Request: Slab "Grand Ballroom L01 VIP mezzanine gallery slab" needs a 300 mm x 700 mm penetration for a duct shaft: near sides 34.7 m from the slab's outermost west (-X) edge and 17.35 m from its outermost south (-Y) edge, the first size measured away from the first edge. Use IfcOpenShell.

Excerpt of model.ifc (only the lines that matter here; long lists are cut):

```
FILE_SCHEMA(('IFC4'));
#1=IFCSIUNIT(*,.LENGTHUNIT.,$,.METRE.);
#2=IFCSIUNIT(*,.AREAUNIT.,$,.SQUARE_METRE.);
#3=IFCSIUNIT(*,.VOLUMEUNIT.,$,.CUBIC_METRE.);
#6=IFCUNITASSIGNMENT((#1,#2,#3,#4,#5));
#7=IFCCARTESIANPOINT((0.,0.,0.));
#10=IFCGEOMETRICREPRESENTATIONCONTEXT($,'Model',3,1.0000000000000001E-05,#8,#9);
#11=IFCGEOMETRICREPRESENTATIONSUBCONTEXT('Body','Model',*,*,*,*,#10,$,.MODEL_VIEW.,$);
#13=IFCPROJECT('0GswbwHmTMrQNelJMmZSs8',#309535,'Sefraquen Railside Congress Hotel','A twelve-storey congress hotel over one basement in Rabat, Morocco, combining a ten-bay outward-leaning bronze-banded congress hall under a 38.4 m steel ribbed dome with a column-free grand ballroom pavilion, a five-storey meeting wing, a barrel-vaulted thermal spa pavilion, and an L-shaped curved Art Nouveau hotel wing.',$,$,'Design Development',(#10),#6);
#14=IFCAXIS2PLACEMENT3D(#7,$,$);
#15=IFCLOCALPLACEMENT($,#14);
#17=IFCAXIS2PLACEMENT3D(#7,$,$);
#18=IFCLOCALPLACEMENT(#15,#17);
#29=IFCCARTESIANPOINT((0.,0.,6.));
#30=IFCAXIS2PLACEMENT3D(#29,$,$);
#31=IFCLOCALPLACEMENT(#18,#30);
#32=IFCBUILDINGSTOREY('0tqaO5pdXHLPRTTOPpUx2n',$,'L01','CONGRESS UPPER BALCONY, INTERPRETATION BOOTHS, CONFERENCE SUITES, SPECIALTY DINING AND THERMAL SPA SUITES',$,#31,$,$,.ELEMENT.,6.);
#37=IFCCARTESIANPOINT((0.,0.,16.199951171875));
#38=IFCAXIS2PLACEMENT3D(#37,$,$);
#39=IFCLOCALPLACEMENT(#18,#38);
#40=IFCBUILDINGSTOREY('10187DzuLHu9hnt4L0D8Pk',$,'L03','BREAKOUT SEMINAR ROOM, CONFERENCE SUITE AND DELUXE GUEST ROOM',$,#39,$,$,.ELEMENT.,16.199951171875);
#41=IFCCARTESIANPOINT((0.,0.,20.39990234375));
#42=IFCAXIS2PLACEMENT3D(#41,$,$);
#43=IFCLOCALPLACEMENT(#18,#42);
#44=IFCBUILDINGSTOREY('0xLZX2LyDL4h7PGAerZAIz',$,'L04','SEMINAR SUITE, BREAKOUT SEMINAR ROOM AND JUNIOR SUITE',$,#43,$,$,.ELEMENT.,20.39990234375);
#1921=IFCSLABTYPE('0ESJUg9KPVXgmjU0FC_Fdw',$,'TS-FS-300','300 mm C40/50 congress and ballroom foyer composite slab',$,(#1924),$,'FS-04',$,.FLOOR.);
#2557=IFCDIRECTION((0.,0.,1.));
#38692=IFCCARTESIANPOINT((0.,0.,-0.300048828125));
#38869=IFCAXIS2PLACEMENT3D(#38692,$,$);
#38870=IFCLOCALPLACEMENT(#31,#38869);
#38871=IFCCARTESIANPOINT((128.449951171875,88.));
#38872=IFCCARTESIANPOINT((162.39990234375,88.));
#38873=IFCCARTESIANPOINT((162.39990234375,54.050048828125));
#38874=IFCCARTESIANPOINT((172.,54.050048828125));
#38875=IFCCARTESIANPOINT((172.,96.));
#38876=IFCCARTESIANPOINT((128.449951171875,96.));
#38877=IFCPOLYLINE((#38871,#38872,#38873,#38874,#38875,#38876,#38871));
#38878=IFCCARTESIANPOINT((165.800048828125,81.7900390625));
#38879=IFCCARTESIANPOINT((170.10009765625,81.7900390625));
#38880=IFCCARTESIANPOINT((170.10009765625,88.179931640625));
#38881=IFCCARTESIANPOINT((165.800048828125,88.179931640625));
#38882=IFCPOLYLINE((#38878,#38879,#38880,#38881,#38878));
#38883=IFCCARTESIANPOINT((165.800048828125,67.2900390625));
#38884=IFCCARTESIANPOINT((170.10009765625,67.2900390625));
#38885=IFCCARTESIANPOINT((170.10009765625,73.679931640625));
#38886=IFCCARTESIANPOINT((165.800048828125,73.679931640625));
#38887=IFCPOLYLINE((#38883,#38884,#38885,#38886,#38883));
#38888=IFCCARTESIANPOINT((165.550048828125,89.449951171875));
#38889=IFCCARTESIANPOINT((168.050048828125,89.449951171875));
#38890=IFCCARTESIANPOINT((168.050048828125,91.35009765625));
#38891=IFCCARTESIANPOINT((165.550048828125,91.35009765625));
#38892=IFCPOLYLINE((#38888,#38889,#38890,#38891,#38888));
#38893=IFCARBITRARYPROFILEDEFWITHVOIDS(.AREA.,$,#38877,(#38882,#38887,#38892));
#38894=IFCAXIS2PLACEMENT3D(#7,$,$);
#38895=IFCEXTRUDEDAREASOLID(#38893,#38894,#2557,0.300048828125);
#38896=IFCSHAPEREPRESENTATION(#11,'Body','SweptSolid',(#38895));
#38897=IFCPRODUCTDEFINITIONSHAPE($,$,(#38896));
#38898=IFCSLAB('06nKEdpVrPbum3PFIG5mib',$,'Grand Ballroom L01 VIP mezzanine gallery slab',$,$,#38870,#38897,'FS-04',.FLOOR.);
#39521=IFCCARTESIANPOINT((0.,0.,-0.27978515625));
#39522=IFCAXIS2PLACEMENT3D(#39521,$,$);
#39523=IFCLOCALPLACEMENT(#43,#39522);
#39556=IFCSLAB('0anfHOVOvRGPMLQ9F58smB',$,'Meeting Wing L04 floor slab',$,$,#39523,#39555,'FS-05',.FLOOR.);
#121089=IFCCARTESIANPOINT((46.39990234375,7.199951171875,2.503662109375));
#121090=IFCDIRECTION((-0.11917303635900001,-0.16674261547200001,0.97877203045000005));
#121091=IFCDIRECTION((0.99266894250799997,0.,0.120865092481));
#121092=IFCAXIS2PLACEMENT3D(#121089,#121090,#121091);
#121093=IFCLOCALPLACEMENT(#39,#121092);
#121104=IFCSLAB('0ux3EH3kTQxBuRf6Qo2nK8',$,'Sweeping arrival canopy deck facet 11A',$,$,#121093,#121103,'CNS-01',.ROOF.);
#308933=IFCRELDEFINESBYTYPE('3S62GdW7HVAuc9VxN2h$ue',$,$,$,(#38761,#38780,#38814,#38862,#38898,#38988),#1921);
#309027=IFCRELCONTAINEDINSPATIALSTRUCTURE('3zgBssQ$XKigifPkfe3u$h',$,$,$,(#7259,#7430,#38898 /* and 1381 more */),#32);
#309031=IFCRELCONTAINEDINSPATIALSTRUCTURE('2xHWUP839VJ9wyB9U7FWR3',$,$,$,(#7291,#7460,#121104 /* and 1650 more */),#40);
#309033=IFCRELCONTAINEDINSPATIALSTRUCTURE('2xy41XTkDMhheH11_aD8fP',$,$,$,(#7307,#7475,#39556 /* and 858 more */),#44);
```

```python
import numpy as np
import ifcopenshell
import ifcopenshell.api.feature
import ifcopenshell.api.geometry
import ifcopenshell.api.root
import ifcopenshell.geom
import ifcopenshell.util.placement
import ifcopenshell.util.representation
import ifcopenshell.util.shape
import ifcopenshell.util.unit

model = ifcopenshell.open("model.ifc")
unit_scale = ifcopenshell.util.unit.calculate_unit_scale(model)
settings = ifcopenshell.geom.settings()


def volume(element):
    """Net volume in cubic metres, openings subtracted."""
    shape = ifcopenshell.geom.create_shape(settings, element)
    return ifcopenshell.util.shape.get_volume(shape.geometry)


slab = model.by_guid("06nKEdpVrPbum3PFIG5mib")
before = volume(slab)

# Extent in the slab's own axes, in metres. The edges named are its -X and -Y sides.
slab_shape = ifcopenshell.geom.create_shape(settings, slab)
vertices = ifcopenshell.util.shape.get_vertices(slab_shape.geometry)
x_min, y_min, bottom = vertices.min(axis=0)
top = vertices[:, 2].max()

opening = ifcopenshell.api.root.create_entity(model, ifc_class="IfcOpeningElement", name="Duct shaft opening", predefined_type="OPENING")
context = ifcopenshell.util.representation.get_context(model, "Model", "Body", "MODEL_VIEW")
width, depth = 0.3, 0.7
outline = [(0.0, 0.0), (width, 0.0), (width, depth), (0.0, depth), (0.0, 0.0)]
# Overshoot both faces by 50 mm so the cut is clean.
shape = ifcopenshell.api.geometry.add_slab_representation(
    model, context=context, depth=top - bottom + 0.1, polyline=outline
)
ifcopenshell.api.geometry.assign_representation(model, product=opening, representation=shape)

matrix = ifcopenshell.util.placement.get_local_placement(slab.ObjectPlacement)
matrix[:, 3] = matrix @ np.append(np.array([x_min + 34.7, y_min + 17.35, bottom - 0.05]) / unit_scale, 1.0)
ifcopenshell.api.geometry.edit_object_placement(model, product=opening, matrix=matrix, is_si=False)
ifcopenshell.api.feature.add_feature(model, feature=opening, element=slab)

after = volume(slab)

print(f"slab volume {before:.3f} -> {after:.3f} m3")

model.write("model_updated.ifc")
```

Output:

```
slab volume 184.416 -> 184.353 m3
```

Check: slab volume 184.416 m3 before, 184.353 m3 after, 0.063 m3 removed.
